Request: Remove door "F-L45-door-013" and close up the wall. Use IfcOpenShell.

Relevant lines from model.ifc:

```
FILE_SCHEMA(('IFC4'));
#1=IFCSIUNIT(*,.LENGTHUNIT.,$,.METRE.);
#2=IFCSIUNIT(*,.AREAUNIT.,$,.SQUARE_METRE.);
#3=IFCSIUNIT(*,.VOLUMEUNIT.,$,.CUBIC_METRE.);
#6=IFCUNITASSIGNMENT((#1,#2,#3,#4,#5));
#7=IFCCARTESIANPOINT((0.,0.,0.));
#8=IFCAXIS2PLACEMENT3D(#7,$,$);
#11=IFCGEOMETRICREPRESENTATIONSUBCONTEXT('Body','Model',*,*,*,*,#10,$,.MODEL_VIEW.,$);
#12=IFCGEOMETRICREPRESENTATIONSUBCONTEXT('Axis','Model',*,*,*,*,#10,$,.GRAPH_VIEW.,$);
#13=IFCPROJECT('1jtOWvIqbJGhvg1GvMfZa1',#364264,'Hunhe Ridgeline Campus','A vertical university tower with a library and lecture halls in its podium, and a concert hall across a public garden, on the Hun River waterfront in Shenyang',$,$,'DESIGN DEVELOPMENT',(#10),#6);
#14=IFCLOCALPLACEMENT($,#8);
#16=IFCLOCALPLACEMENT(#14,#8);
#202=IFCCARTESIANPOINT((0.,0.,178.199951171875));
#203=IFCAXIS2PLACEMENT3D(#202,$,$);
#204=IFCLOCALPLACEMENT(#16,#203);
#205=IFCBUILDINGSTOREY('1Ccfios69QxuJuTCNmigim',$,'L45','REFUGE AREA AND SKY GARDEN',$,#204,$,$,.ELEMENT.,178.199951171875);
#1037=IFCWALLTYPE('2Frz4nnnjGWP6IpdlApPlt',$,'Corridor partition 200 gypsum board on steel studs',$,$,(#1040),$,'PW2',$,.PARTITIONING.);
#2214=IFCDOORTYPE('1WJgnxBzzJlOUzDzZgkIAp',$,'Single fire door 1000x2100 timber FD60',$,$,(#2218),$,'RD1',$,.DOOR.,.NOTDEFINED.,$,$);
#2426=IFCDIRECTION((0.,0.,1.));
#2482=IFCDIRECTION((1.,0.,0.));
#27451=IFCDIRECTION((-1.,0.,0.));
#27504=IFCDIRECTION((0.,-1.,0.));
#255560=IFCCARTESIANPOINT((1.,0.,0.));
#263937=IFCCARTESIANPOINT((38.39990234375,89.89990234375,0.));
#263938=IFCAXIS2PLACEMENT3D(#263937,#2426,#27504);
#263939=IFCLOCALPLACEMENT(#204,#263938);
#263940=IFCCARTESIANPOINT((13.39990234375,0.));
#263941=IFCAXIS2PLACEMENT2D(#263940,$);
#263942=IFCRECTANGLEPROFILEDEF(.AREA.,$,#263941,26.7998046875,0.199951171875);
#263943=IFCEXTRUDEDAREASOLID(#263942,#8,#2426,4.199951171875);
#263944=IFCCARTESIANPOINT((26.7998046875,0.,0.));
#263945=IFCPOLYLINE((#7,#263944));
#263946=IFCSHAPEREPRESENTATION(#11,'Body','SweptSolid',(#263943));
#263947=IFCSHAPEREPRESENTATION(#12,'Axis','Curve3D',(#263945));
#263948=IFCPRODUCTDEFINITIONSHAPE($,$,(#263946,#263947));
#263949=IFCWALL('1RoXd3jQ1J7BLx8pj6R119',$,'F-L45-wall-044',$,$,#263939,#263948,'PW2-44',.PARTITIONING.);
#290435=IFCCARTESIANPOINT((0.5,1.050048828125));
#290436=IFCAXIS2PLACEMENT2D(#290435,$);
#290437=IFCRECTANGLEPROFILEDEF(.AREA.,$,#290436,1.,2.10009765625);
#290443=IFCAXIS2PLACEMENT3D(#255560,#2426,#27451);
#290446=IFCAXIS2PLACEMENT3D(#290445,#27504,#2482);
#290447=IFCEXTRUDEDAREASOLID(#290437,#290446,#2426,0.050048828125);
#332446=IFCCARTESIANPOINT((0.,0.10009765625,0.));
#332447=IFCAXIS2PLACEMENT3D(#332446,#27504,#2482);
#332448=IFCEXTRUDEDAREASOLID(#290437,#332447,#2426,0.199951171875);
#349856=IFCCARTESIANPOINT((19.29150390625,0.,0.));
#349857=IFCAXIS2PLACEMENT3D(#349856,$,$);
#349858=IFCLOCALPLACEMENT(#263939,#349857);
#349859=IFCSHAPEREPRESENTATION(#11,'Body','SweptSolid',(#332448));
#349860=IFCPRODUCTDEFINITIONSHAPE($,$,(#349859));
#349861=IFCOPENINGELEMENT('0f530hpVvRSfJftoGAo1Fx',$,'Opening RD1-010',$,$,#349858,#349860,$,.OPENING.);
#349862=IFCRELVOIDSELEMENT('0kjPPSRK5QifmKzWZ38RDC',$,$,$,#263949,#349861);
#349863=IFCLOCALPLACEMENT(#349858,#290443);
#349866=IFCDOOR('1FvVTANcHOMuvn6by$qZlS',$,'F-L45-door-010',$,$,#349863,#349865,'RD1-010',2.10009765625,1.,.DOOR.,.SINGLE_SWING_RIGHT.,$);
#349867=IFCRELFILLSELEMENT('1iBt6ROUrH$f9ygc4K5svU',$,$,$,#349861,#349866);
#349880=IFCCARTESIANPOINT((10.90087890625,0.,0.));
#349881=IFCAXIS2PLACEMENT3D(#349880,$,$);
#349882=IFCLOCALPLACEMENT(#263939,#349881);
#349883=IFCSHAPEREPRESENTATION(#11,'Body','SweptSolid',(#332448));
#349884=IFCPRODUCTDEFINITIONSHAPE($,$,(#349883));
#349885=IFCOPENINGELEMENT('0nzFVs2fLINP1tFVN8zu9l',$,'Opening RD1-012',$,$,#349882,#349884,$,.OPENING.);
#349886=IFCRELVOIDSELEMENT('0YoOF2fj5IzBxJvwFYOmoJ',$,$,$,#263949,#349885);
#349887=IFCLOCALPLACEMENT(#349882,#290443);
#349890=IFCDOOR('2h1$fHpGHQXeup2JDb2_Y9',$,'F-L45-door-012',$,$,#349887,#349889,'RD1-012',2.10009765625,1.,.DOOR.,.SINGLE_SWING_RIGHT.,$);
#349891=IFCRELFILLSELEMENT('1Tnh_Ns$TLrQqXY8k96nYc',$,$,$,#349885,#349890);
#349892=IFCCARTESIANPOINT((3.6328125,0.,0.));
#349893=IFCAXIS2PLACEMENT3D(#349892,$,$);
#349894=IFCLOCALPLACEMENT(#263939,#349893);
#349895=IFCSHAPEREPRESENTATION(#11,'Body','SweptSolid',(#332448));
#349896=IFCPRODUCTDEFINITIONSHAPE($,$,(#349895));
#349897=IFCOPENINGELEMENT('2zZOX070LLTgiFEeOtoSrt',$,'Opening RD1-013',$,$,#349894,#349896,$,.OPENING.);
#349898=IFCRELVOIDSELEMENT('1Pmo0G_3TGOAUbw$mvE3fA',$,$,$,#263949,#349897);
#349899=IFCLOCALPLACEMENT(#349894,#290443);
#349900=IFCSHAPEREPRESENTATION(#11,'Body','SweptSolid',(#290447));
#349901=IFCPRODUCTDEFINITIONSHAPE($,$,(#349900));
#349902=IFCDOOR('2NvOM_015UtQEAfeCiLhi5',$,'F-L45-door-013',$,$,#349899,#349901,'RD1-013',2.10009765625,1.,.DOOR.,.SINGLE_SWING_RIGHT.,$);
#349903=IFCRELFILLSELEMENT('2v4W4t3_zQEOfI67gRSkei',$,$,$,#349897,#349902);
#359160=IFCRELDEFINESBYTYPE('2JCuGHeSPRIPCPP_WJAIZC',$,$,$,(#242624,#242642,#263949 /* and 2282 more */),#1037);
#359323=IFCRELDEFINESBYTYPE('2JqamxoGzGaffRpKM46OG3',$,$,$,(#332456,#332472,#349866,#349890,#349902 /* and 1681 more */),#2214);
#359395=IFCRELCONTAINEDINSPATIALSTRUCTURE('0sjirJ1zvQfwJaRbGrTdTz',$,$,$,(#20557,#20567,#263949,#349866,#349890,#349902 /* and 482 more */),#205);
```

```python
import ifcopenshell
import ifcopenshell.api.feature
import ifcopenshell.api.root
import ifcopenshell.geom
import ifcopenshell.util.shape

model = ifcopenshell.open("model.ifc")
settings = ifcopenshell.geom.settings()


def volume(element):
    """Net volume in cubic metres, openings subtracted."""
    shape = ifcopenshell.geom.create_shape(settings, element)
    return ifcopenshell.util.shape.get_volume(shape.geometry)


door = model.by_guid("2NvOM_015UtQEAfeCiLhi5")
opening = door.FillsVoids[0].RelatingOpeningElement
wall = opening.VoidsElements[0].RelatingBuildingElement
before = volume(wall)

ifcopenshell.api.root.remove_product(model, product=door)
ifcopenshell.api.feature.remove_feature(model, feature=opening)

after = volume(wall)

print(f"wall volume {before:.3f} -> {after:.3f} m3")

model.write("model_rev.ifc")
```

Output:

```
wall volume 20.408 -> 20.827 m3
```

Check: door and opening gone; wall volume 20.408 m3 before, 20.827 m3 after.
